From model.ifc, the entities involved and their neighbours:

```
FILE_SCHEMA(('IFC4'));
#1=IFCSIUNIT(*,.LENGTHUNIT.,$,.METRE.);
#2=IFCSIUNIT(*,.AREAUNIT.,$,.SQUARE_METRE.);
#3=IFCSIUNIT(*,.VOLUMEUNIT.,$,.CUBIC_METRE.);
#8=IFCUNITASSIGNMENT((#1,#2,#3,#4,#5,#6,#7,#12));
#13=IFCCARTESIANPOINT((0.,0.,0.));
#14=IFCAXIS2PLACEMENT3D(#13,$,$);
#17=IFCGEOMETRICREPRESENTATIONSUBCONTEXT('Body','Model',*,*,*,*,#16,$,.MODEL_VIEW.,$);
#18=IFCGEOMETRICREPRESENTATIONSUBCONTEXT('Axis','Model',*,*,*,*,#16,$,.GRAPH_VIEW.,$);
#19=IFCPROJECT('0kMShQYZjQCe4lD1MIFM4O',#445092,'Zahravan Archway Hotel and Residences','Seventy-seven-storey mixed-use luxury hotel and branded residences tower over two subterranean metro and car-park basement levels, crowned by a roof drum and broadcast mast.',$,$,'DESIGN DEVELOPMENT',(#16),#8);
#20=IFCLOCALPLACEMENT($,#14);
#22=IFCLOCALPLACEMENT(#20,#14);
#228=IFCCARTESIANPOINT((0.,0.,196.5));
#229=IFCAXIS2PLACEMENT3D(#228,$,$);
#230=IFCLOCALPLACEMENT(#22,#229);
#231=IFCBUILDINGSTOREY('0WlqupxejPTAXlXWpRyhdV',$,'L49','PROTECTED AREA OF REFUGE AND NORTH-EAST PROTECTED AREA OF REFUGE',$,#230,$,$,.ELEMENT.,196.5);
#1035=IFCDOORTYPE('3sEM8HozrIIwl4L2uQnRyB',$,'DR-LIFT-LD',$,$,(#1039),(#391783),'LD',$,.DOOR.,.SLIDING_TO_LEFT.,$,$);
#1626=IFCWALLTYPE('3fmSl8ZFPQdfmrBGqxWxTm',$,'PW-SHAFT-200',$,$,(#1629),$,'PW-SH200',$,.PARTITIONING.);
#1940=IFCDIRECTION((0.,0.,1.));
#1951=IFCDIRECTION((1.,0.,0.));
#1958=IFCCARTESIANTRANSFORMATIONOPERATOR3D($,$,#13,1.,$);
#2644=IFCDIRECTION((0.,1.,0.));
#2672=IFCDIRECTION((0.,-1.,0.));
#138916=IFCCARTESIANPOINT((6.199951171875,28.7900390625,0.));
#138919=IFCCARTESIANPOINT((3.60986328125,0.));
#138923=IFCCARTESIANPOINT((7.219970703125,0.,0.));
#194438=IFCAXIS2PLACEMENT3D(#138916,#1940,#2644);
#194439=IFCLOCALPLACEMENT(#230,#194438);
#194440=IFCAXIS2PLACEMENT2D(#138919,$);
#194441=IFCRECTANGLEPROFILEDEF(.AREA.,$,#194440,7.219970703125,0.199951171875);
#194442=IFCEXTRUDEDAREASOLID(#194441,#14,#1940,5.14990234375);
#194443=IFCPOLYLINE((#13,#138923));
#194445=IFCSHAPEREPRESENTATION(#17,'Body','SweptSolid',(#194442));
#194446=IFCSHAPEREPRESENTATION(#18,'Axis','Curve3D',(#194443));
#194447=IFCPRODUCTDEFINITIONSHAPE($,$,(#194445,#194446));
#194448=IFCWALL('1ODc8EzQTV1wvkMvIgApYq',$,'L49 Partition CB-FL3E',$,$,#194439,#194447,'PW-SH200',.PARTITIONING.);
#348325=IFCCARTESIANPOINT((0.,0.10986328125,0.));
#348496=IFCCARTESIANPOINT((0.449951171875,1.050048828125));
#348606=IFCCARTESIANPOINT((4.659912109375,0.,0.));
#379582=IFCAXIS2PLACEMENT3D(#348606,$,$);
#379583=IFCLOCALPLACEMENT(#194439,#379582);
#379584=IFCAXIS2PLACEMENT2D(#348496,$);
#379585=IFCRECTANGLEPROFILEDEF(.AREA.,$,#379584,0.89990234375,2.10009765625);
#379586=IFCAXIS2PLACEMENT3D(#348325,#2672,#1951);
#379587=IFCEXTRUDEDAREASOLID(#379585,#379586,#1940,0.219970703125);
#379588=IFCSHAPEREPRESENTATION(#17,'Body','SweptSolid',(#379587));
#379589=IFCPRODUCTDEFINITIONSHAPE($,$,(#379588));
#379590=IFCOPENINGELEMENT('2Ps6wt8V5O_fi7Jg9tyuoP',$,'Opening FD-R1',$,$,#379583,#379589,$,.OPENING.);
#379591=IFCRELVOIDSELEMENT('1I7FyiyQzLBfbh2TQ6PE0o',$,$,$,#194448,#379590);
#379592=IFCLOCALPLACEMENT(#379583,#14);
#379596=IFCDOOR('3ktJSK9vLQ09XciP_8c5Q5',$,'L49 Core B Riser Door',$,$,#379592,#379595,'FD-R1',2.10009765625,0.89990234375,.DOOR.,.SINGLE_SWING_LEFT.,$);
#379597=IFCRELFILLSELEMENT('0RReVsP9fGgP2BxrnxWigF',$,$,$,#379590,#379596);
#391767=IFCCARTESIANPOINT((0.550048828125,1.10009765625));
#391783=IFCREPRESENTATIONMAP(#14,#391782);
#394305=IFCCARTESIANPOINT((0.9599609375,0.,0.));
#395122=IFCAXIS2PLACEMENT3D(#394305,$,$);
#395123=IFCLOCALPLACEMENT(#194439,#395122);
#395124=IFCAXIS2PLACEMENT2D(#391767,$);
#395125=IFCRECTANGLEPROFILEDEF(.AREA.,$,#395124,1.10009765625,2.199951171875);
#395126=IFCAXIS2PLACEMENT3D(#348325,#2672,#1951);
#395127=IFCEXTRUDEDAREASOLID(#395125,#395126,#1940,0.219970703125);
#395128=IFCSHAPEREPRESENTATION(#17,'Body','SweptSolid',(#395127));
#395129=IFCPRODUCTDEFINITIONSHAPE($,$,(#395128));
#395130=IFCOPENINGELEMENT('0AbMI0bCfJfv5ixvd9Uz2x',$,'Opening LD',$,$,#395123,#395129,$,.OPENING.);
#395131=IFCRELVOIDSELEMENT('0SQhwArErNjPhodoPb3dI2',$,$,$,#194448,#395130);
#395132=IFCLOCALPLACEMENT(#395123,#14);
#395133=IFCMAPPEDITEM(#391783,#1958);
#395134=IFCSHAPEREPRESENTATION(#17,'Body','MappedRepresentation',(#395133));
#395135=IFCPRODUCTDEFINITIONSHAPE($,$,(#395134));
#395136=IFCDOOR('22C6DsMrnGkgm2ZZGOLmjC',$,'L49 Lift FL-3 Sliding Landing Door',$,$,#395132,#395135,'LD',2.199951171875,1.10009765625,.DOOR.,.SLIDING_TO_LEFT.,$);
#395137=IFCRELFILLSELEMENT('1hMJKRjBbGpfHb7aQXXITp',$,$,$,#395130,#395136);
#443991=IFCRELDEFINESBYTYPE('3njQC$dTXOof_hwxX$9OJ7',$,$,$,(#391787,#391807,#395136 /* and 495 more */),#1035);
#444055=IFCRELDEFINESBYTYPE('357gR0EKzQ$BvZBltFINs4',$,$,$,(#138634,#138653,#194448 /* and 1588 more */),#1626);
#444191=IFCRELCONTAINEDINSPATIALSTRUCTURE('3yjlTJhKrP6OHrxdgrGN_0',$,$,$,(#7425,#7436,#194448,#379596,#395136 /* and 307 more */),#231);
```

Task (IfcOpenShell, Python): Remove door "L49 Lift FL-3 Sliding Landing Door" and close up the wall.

```python
import ifcopenshell
import ifcopenshell.api.feature
import ifcopenshell.api.root
import ifcopenshell.geom
import ifcopenshell.util.shape

model = ifcopenshell.open("model.ifc")
settings = ifcopenshell.geom.settings()


def volume(element):
    """Net volume in cubic metres, openings subtracted."""
    shape = ifcopenshell.geom.create_shape(settings, element)
    return ifcopenshell.util.shape.get_volume(shape.geometry)


door = model.by_id(395136)
opening = door.FillsVoids[0].RelatingOpeningElement
wall = opening.VoidsElements[0].RelatingBuildingElement
before = volume(wall)

ifcopenshell.api.root.remove_product(model, product=door)
ifcopenshell.api.feature.remove_feature(model, feature=opening)

after = volume(wall)

print(f"wall volume {before:.3f} -> {after:.3f} m3")

model.write("model_v2.ifc")
```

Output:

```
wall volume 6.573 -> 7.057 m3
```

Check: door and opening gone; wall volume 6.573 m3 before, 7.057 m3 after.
